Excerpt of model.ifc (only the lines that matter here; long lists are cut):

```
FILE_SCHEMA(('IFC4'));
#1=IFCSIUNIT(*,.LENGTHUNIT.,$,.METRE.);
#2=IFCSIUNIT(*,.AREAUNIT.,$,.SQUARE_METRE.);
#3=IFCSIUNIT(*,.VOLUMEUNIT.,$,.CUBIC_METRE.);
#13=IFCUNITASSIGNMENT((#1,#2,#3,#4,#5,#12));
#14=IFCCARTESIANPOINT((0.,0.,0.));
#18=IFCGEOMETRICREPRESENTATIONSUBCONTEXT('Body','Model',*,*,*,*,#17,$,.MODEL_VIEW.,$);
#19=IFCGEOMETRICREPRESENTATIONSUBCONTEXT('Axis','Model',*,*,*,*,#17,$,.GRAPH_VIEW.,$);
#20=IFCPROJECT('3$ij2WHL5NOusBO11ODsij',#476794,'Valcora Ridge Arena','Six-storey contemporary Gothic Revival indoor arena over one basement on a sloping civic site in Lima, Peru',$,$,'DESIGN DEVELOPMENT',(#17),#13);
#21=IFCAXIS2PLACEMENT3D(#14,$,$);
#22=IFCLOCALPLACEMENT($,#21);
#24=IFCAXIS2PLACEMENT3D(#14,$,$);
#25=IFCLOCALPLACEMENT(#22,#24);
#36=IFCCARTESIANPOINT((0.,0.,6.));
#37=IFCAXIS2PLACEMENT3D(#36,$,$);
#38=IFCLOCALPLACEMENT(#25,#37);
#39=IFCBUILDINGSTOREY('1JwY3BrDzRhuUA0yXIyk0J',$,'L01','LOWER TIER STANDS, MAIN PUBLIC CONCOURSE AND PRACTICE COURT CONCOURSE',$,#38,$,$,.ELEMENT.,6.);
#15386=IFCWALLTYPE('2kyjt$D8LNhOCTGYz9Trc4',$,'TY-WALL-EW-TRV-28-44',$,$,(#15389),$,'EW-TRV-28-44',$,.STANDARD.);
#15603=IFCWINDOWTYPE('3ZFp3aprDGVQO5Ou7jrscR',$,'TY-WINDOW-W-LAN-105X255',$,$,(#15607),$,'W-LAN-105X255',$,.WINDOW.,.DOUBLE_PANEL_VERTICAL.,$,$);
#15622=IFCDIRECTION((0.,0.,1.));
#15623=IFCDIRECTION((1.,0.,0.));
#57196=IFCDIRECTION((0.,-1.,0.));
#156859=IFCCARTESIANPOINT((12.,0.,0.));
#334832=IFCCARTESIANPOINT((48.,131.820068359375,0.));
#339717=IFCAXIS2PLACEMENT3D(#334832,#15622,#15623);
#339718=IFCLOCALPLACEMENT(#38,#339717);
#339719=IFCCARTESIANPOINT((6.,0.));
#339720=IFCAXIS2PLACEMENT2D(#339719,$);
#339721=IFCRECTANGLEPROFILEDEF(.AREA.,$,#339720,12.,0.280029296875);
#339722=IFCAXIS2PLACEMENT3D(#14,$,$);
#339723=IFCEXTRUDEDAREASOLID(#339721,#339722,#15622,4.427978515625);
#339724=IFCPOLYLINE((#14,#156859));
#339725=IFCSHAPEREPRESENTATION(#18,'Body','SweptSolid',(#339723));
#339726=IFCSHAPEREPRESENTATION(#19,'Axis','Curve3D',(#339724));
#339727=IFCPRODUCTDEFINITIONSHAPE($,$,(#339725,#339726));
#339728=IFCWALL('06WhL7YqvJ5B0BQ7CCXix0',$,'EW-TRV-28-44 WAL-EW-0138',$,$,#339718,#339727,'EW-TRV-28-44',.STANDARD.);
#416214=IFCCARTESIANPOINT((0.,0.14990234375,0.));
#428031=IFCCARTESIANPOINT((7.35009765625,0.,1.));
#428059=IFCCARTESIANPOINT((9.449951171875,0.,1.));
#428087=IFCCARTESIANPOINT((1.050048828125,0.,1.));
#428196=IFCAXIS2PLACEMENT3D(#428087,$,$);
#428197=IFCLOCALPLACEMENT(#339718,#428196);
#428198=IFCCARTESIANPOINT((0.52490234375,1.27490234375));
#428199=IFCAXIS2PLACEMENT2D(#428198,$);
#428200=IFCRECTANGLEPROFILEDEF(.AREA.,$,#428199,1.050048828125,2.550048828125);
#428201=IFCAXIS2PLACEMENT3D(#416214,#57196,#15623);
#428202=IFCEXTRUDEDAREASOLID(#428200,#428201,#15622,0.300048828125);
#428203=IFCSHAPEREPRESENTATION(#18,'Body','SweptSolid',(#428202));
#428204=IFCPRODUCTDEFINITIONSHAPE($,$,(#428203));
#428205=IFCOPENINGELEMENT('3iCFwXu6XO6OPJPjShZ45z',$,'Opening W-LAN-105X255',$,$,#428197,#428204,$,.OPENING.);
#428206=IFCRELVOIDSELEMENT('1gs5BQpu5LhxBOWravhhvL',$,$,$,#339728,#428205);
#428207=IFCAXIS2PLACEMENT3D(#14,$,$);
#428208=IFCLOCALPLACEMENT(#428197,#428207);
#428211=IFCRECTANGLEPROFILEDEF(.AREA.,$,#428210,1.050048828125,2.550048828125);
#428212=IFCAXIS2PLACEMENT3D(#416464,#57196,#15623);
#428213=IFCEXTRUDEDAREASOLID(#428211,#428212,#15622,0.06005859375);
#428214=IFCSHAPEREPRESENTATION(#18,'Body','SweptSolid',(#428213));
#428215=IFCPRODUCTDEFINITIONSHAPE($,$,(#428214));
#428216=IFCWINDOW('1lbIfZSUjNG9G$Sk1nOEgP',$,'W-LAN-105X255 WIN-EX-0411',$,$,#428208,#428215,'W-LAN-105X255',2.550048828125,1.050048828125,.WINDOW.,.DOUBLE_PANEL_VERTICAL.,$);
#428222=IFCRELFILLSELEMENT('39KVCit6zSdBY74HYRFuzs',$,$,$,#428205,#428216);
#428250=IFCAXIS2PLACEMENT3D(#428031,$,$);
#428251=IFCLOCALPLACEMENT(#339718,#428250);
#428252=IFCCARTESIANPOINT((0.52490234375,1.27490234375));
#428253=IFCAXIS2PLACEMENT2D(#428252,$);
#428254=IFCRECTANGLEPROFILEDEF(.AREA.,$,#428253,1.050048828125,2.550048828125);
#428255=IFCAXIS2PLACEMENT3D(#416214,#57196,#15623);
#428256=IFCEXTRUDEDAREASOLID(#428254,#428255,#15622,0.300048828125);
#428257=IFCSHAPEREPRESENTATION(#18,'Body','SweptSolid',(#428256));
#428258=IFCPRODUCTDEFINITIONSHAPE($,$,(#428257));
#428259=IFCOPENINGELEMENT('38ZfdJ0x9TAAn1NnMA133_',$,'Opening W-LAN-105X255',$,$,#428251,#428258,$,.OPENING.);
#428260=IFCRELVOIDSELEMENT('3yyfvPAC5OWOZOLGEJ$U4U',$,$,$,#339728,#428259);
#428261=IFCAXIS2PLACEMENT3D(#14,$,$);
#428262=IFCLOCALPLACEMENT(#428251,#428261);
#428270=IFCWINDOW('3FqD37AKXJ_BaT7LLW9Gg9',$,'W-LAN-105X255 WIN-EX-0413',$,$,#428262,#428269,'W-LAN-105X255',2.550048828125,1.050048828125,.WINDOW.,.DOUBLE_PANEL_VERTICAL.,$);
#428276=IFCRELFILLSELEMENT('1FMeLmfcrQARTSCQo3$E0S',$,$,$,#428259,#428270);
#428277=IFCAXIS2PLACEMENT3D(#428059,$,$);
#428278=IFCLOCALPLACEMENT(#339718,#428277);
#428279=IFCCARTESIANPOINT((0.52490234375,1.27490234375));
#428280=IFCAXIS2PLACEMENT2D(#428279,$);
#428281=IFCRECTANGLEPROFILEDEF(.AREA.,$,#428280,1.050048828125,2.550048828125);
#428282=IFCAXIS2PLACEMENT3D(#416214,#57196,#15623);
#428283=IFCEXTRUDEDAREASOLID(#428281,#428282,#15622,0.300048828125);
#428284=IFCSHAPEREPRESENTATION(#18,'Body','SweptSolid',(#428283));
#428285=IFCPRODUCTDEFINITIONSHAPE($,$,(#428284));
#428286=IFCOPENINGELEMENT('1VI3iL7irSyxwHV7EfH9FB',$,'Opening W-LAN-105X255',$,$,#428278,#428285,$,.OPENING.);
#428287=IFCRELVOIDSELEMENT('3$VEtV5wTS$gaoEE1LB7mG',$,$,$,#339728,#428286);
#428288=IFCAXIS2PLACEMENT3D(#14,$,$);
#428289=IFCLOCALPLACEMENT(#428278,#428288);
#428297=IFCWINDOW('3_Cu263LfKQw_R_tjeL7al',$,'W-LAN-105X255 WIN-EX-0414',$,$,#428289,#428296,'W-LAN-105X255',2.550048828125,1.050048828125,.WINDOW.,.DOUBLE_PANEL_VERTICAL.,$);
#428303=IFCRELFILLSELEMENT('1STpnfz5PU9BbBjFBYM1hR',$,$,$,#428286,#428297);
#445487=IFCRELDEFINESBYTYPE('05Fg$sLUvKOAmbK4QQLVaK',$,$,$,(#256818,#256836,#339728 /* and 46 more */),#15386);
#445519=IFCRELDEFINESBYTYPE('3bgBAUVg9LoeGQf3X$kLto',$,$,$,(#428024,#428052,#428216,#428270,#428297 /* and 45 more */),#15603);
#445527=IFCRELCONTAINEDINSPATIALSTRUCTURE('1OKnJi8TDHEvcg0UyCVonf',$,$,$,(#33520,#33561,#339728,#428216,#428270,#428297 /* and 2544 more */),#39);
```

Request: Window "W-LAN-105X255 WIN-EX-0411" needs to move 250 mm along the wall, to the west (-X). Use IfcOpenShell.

```python
import ifcopenshell
import ifcopenshell.api.geometry
import ifcopenshell.util.placement
import ifcopenshell.util.unit

model = ifcopenshell.open("model.ifc")
unit_scale = ifcopenshell.util.unit.calculate_unit_scale(model)

window = model.by_guid("1lbIfZSUjNG9G$Sk1nOEgP")
opening = window.FillsVoids[0].RelatingOpeningElement
wall = opening.VoidsElements[0].RelatingBuildingElement

wall_matrix = ifcopenshell.util.placement.get_local_placement(wall.ObjectPlacement)
shift = wall_matrix[:3, 0] * -0.25 / unit_scale
before = ifcopenshell.util.placement.get_local_placement(window.ObjectPlacement)[:3, 3].copy()

# The window is placed relative to its opening, so it follows when the opening moves.
matrix = ifcopenshell.util.placement.get_local_placement(opening.ObjectPlacement)
matrix[:3, 3] += shift
ifcopenshell.api.geometry.edit_object_placement(
    model, product=opening, matrix=matrix, is_si=False, should_transform_children=True
)

after = ifcopenshell.util.placement.get_local_placement(window.ObjectPlacement)[:3, 3]
print("window moved by", (after - before).round(3) + 0.0)

model.write("model_rev.ifc")
```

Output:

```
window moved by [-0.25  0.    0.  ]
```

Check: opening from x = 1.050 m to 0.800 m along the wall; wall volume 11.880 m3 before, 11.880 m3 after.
